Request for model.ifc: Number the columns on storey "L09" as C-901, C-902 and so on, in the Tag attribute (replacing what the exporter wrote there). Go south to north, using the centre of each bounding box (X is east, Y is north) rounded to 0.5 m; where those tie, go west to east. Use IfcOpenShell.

First a look at what the model holds.

```python
import ifcopenshell
import ifcopenshell.util.element
import ifcopenshell.util.placement

model = ifcopenshell.open("model.ifc")
print(model.schema)
storey = next(s for s in model.by_type("IfcBuildingStorey") if s.Name == "L09")
columns = [e for e in ifcopenshell.util.element.get_decomposition(storey) if e.is_a("IfcColumn")]
for e in sorted(columns, key=lambda e: e.id()):
    origin = ifcopenshell.util.placement.get_local_placement(e.ObjectPlacement)[:3, 3]
    print(e.id(), e.Tag, e.Name, origin.round(2) + 0.0, sep=" | ")
```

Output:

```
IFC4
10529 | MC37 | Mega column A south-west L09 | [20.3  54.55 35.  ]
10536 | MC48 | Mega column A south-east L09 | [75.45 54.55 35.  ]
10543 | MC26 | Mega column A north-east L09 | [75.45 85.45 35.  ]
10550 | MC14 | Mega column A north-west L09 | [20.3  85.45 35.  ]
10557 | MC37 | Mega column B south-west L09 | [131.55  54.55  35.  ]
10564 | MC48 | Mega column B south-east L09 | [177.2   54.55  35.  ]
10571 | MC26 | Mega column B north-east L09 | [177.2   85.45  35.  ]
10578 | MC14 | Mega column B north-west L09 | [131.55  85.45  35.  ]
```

```python
import ifcopenshell
import ifcopenshell.geom
import ifcopenshell.util.element
import ifcopenshell.util.shape

model = ifcopenshell.open("model.ifc")
settings = ifcopenshell.geom.settings()
settings.set("use-world-coords", True)


def centre(element):
    shape = ifcopenshell.geom.create_shape(settings, element)
    return ifcopenshell.util.shape.get_bbox_centroid(shape.geometry)


storey = next(s for s in model.by_type("IfcBuildingStorey") if s.Name == "L09")
columns = [e for e in ifcopenshell.util.element.get_decomposition(storey) if e.is_a("IfcColumn")]

# Insertion points can sit at a corner or the storey origin, so sort by the geometry (in metres).
centres = {e: centre(e) for e in columns}
columns.sort(key=lambda e: (round(centres[e][1] / 0.5), centres[e][0]))

for i, e in enumerate(columns, start=1):
    number = f"C-9{i:02d}"
    e.Tag = number
    print(e.id(), number)

model.write("model_updated.ifc")
```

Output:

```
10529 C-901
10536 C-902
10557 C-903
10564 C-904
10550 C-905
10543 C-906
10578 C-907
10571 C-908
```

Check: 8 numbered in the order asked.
